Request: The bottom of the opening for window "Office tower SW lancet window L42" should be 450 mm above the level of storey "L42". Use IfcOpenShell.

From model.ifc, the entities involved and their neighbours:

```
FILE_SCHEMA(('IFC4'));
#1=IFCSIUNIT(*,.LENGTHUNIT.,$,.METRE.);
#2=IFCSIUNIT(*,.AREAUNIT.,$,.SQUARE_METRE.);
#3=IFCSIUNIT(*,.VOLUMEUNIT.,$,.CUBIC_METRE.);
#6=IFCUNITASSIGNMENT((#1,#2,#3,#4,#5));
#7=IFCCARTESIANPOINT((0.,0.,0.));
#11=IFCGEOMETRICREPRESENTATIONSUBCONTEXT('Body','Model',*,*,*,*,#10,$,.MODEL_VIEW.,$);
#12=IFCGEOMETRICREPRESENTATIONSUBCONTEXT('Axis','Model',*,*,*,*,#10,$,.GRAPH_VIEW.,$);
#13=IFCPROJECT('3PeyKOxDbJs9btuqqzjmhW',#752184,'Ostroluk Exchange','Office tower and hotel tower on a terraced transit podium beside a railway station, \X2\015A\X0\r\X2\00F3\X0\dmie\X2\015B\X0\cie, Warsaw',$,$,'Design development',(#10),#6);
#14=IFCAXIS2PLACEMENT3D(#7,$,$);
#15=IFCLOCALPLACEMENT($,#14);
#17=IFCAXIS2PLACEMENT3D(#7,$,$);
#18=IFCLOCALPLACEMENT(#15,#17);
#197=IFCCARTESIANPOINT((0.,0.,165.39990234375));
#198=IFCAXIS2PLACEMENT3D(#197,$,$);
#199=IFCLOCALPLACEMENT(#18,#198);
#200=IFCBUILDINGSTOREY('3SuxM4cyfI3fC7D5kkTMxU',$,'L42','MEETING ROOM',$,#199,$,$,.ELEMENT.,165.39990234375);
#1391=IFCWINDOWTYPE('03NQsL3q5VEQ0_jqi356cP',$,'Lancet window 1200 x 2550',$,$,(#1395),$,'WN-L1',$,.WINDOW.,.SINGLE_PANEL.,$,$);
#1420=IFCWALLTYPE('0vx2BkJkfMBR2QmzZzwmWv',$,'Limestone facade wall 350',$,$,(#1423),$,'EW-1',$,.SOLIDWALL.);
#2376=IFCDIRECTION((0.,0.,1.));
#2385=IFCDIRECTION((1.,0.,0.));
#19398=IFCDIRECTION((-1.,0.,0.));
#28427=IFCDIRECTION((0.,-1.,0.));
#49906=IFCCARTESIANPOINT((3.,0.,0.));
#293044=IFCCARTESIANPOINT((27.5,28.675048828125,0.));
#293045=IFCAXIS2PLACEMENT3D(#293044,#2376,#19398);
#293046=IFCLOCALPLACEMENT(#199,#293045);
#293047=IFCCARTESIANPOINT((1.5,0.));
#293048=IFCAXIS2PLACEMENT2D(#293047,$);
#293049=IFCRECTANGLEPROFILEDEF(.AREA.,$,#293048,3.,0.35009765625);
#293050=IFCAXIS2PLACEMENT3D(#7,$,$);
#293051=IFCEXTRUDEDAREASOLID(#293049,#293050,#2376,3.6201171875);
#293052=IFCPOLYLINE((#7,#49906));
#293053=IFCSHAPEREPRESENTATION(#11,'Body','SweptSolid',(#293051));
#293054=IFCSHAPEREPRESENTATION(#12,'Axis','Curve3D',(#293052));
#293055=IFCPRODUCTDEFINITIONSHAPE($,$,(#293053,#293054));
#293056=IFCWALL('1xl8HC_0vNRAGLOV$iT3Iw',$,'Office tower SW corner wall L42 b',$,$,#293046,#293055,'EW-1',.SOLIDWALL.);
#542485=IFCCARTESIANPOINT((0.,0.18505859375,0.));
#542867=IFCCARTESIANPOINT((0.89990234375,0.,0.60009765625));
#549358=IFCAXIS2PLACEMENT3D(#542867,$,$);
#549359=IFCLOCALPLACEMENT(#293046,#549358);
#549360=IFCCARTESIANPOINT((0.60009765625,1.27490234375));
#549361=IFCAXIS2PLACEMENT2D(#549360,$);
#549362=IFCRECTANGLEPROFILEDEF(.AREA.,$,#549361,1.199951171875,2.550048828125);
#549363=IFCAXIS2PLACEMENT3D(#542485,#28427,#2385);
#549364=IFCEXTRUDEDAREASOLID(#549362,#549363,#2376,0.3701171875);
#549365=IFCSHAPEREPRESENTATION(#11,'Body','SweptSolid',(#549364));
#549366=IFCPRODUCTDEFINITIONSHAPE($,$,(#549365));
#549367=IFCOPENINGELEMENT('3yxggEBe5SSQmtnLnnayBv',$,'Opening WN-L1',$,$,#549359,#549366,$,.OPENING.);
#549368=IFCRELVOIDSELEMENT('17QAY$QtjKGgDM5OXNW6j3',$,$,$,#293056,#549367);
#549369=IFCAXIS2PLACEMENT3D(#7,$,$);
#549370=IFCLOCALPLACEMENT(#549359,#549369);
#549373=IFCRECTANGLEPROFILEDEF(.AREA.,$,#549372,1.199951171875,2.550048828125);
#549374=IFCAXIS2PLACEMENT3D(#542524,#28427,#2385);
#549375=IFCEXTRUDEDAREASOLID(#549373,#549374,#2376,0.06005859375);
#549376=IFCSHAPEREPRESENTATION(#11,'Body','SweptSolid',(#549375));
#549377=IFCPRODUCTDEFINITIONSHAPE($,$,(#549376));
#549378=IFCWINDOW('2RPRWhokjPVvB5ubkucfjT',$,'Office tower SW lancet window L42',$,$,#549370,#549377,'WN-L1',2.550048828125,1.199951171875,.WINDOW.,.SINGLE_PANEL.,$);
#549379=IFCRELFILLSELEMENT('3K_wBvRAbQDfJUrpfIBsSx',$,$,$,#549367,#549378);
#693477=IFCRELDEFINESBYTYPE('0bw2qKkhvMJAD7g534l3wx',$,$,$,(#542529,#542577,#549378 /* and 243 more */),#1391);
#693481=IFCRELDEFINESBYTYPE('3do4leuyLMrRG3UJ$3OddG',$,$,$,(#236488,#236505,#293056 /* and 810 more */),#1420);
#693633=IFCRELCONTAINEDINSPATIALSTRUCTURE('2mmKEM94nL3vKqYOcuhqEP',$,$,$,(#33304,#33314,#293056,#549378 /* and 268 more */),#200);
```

```python
import numpy as np
import ifcopenshell
import ifcopenshell.api.geometry
import ifcopenshell.geom
import ifcopenshell.util.element
import ifcopenshell.util.placement
import ifcopenshell.util.shape
import ifcopenshell.util.unit

model = ifcopenshell.open("model.ifc")
unit_scale = ifcopenshell.util.unit.calculate_unit_scale(model)

window = model.by_guid("2RPRWhokjPVvB5ubkucfjT")
opening = window.FillsVoids[0].RelatingOpeningElement
storey = ifcopenshell.util.element.get_container(window, ifc_class="IfcBuildingStorey")
level = ifcopenshell.util.placement.get_local_placement(storey.ObjectPlacement)[2, 3]

# The opening's origin need not be at the sill, so measure its lowest point.
shape = ifcopenshell.geom.create_shape(ifcopenshell.geom.settings(), opening)
bottom = ifcopenshell.util.shape.get_shape_bottom_elevation(shape, shape.geometry) / unit_scale
dz = level + 0.45 / unit_scale - bottom

shift = np.array([0.0, 0.0, dz])
# The window is placed relative to its opening, so it follows when the opening moves.
matrix = ifcopenshell.util.placement.get_local_placement(opening.ObjectPlacement)
matrix[:3, 3] += shift
ifcopenshell.api.geometry.edit_object_placement(
    model, product=opening, matrix=matrix, is_si=False, should_transform_children=True
)

print(f"moved by {dz * unit_scale:+.3f} m")

model.write("model_updated.ifc")
```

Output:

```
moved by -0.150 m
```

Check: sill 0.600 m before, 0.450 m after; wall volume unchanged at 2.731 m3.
